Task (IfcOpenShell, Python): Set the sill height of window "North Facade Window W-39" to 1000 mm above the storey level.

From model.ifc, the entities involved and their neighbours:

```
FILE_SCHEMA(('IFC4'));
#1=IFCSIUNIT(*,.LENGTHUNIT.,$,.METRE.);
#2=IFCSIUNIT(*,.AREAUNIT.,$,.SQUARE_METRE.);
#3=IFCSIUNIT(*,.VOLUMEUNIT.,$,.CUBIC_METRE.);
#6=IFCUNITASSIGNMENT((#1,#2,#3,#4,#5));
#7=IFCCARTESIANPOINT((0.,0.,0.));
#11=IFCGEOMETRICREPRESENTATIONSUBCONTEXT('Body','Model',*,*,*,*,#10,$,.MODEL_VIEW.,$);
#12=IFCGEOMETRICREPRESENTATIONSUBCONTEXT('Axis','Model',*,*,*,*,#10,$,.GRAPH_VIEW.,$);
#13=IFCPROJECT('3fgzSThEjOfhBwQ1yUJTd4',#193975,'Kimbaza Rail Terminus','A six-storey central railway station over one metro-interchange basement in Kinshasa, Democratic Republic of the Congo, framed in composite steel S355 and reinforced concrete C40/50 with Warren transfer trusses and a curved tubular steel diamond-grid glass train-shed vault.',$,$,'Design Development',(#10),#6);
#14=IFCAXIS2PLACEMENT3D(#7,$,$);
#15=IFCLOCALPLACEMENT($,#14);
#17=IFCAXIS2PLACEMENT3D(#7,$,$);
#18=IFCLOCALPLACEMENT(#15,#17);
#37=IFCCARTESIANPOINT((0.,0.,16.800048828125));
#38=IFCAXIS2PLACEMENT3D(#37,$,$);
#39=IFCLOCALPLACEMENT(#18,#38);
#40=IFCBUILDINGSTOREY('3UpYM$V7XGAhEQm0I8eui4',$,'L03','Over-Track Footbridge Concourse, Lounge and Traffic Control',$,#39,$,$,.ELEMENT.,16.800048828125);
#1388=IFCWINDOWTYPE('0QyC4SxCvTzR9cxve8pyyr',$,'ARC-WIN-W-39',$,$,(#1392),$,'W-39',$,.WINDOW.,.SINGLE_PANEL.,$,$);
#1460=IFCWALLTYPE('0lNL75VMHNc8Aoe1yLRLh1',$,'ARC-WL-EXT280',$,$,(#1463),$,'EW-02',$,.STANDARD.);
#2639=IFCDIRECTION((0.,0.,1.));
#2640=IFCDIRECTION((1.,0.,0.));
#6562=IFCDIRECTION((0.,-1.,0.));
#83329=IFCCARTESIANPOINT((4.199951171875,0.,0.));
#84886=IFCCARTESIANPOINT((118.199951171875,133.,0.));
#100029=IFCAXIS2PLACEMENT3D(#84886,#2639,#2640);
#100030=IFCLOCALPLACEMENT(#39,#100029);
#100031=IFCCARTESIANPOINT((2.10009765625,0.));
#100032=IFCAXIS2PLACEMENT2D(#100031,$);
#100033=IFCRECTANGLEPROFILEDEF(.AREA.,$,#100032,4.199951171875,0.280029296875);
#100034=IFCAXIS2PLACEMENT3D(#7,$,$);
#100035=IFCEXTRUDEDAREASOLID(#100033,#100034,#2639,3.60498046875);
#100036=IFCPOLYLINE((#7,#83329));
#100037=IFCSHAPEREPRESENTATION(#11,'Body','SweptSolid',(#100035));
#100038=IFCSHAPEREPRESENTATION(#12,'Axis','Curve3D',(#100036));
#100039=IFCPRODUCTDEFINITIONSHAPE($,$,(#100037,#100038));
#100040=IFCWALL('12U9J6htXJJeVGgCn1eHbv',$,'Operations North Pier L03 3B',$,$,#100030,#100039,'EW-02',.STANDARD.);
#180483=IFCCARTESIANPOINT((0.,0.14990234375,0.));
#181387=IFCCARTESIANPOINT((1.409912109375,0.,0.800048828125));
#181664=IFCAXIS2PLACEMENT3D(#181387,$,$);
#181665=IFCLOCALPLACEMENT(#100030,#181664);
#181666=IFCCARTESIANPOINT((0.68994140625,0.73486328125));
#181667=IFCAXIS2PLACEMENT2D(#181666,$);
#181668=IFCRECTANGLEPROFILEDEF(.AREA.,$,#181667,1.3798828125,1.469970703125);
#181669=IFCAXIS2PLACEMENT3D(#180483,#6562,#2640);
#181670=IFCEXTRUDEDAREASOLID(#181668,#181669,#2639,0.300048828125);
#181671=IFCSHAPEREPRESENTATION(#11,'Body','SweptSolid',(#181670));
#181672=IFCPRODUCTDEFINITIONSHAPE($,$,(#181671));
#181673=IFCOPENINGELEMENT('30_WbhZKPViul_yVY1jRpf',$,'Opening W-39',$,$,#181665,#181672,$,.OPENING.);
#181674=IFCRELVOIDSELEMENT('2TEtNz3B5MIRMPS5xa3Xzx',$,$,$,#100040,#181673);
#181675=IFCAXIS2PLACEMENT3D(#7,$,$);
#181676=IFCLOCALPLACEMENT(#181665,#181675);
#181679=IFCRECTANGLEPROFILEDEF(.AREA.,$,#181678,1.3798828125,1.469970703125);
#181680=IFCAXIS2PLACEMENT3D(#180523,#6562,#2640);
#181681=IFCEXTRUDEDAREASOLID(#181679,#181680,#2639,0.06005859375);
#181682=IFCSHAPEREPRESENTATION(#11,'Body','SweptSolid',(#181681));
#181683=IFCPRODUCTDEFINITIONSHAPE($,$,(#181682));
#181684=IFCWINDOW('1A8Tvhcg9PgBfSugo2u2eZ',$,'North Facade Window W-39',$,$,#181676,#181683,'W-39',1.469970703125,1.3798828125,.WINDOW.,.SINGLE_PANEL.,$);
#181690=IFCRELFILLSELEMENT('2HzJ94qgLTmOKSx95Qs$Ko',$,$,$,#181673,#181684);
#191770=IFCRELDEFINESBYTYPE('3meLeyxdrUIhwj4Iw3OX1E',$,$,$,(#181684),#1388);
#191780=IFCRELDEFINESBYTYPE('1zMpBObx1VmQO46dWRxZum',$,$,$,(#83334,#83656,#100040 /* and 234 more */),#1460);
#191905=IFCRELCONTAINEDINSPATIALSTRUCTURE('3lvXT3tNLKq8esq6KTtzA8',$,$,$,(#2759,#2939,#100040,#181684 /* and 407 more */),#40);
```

```python
import numpy as np
import ifcopenshell
import ifcopenshell.api.geometry
import ifcopenshell.geom
import ifcopenshell.util.element
import ifcopenshell.util.placement
import ifcopenshell.util.shape
import ifcopenshell.util.unit

model = ifcopenshell.open("model.ifc")
unit_scale = ifcopenshell.util.unit.calculate_unit_scale(model)

window = model.by_guid("1A8Tvhcg9PgBfSugo2u2eZ")
opening = window.FillsVoids[0].RelatingOpeningElement
storey = ifcopenshell.util.element.get_container(window, ifc_class="IfcBuildingStorey")
level = ifcopenshell.util.placement.get_local_placement(storey.ObjectPlacement)[2, 3]

# The opening's origin need not be at the sill, so measure its lowest point.
shape = ifcopenshell.geom.create_shape(ifcopenshell.geom.settings(), opening)
bottom = ifcopenshell.util.shape.get_shape_bottom_elevation(shape, shape.geometry) / unit_scale
dz = level + 1 / unit_scale - bottom

shift = np.array([0.0, 0.0, dz])
# The window is placed relative to its opening, so it follows when the opening moves.
matrix = ifcopenshell.util.placement.get_local_placement(opening.ObjectPlacement)
matrix[:3, 3] += shift
ifcopenshell.api.geometry.edit_object_placement(
    model, product=opening, matrix=matrix, is_si=False, should_transform_children=True
)

print(f"moved by {dz * unit_scale:+.3f} m")

model.write("model_edited.ifc")
```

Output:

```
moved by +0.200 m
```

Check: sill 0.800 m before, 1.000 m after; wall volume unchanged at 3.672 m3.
